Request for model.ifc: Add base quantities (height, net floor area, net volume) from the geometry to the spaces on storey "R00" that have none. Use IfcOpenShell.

First a look at what the model holds.

```python
import ifcopenshell
import ifcopenshell.util.element
import ifcopenshell.util.unit

model = ifcopenshell.open("model.ifc")
print(model.schema)
for unit_type in ("LENGTHUNIT", "AREAUNIT", "VOLUMEUNIT"):
    print(unit_type, ifcopenshell.util.unit.calculate_unit_scale(model, unit_type))
storey = next(s for s in model.by_type("IfcBuildingStorey") if s.Name == "R00")
spaces = [e for e in ifcopenshell.util.element.get_decomposition(storey) if e.is_a("IfcSpace")]
for e in sorted(spaces, key=lambda e: e.id()):
    print(e.id(), e.is_a(), e.Name, list(ifcopenshell.util.element.get_psets(e, qtos_only=True)), sep=" | ")
```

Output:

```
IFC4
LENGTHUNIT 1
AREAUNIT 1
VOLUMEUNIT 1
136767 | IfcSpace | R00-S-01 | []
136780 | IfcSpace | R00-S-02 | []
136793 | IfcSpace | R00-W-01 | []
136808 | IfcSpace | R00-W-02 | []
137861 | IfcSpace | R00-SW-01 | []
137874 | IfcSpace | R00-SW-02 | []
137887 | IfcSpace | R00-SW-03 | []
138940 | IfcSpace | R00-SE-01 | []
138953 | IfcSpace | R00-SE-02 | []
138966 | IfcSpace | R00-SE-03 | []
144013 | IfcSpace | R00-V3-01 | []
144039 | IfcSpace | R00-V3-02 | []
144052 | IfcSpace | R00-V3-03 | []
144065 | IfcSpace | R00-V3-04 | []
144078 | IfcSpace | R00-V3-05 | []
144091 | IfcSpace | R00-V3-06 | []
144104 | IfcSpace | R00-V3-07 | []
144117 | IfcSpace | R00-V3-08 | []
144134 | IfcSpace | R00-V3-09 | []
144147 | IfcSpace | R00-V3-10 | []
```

```python
import ifcopenshell
import ifcopenshell.api.pset
import ifcopenshell.geom
import ifcopenshell.util.element
import ifcopenshell.util.shape
import ifcopenshell.util.unit

model = ifcopenshell.open("model.ifc")
unit_scale = ifcopenshell.util.unit.calculate_unit_scale(model)
area_scale = ifcopenshell.util.unit.calculate_unit_scale(model, "AREAUNIT")
volume_scale = ifcopenshell.util.unit.calculate_unit_scale(model, "VOLUMEUNIT")
settings = ifcopenshell.geom.settings()

storey = next(s for s in model.by_type("IfcBuildingStorey") if s.Name == "R00")
spaces = [e for e in ifcopenshell.util.element.get_decomposition(storey) if e.is_a("IfcSpace")]

for e in sorted(spaces, key=lambda e: e.id()):
    if ifcopenshell.util.element.get_psets(e, qtos_only=True, should_inherit=False):
        continue
    # Geometry comes back in metres, in the element's own axes.
    shape = ifcopenshell.geom.create_shape(settings, e)
    values = {
        "Height": ifcopenshell.util.shape.get_z(shape.geometry) / unit_scale,
        "NetFloorArea": ifcopenshell.util.shape.get_footprint_area(shape.geometry) / area_scale,
        "NetVolume": ifcopenshell.util.shape.get_volume(shape.geometry) / volume_scale,
    }
    qto = ifcopenshell.api.pset.add_qto(model, product=e, name="Qto_SpaceBaseQuantities")
    ifcopenshell.api.pset.edit_qto(model, qto=qto, properties=values)
    print(e.id(), {k: round(v, 3) for k, v in values.items()})

model.write("model_updated.ifc")
```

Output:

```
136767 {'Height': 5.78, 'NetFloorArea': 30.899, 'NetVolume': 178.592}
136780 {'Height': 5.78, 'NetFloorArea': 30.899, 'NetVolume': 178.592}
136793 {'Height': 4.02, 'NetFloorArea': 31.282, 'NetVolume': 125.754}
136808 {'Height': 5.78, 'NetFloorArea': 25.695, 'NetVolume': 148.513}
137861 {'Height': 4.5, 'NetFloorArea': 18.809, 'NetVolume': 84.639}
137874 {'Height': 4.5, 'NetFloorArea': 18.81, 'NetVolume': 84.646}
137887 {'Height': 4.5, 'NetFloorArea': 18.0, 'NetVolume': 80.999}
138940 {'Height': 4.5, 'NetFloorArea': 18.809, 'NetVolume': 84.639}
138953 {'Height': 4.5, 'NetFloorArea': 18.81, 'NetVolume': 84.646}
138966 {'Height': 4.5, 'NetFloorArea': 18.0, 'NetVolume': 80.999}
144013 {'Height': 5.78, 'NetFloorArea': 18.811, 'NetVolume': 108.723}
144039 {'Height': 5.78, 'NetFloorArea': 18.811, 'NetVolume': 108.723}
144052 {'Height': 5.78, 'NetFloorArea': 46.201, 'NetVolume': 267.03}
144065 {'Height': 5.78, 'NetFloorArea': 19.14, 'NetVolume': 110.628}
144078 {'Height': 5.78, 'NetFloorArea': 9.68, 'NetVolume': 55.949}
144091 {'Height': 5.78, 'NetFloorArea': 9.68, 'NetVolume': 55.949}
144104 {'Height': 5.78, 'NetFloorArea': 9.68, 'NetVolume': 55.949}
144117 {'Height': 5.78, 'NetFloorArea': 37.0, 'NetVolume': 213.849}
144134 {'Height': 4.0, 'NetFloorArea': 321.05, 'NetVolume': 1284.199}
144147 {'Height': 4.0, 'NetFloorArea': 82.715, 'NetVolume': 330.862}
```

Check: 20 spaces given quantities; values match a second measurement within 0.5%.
